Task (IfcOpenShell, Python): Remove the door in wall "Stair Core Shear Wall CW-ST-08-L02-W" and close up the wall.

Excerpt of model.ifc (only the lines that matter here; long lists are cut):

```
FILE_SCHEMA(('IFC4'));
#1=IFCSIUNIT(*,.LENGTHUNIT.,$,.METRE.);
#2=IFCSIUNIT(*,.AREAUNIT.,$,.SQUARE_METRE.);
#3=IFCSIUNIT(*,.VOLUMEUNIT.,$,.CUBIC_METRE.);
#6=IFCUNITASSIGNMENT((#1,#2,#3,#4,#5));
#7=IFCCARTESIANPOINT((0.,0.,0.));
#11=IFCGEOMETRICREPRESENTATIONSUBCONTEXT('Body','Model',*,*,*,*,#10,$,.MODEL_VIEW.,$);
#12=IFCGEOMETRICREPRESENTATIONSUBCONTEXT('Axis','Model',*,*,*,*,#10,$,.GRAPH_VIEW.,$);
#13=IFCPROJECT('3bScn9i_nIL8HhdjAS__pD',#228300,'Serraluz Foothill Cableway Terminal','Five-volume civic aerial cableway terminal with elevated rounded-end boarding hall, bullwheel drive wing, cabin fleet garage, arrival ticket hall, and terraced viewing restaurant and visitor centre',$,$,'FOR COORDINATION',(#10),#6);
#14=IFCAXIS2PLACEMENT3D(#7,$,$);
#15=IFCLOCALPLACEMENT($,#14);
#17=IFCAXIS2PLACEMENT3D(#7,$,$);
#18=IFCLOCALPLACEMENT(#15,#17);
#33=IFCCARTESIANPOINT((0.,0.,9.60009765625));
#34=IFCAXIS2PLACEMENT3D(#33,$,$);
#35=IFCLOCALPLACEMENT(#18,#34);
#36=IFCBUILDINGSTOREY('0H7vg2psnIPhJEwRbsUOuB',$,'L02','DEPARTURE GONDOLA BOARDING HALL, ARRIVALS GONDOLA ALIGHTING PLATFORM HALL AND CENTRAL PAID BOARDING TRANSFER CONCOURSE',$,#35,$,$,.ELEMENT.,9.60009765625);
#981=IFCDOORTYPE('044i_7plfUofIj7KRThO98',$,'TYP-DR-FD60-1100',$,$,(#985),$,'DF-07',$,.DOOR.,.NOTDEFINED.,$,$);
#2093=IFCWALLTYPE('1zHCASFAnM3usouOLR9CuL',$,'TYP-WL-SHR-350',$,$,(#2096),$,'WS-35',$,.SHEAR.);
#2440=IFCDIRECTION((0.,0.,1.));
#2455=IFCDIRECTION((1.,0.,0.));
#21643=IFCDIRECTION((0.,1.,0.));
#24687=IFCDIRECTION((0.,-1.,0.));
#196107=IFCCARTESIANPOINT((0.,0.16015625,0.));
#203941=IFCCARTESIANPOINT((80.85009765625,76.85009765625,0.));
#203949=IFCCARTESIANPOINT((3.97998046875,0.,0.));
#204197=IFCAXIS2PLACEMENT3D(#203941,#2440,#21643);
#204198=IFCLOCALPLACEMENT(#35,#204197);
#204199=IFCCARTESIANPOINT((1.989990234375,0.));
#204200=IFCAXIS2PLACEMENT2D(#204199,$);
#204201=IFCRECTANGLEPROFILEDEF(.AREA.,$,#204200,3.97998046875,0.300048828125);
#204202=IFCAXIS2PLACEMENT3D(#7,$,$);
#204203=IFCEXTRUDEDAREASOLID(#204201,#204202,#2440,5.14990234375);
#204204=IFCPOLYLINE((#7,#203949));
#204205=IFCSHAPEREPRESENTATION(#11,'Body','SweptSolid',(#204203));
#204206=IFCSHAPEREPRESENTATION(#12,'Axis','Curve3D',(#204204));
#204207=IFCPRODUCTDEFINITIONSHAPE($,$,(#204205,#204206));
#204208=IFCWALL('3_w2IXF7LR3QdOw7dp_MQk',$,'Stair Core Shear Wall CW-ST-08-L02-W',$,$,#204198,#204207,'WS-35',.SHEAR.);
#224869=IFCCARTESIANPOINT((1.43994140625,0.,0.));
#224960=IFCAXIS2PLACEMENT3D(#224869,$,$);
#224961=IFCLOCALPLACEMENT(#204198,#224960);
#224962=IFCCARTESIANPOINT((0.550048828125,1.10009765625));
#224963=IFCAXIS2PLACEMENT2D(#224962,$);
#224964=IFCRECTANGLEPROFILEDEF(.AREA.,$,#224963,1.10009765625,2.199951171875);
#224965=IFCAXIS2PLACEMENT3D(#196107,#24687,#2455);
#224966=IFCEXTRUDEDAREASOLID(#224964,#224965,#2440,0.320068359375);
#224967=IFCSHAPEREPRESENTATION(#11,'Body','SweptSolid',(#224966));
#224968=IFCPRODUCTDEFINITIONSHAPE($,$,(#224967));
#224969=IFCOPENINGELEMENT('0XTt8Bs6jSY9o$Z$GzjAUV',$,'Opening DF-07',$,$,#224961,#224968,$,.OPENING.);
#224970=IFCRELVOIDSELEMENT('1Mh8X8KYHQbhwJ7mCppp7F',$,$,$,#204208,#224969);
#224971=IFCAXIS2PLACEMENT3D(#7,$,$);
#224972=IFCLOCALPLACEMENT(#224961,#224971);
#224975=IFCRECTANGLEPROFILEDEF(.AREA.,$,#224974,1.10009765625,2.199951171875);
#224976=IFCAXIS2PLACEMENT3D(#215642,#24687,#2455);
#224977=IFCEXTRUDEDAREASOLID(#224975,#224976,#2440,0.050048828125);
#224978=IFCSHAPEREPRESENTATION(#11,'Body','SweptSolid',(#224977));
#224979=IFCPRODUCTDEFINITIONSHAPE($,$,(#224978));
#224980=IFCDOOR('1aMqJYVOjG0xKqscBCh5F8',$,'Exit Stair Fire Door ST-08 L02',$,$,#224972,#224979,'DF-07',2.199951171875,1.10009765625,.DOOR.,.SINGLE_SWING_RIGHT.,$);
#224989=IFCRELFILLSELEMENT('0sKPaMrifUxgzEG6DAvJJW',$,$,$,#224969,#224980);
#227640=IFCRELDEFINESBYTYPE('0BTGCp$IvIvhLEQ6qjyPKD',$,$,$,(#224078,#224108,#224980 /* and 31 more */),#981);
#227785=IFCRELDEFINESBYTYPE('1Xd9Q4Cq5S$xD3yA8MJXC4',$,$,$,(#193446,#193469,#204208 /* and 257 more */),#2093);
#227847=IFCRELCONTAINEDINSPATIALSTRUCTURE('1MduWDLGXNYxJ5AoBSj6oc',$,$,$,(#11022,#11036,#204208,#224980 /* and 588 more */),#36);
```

```python
import ifcopenshell
import ifcopenshell.api.feature
import ifcopenshell.api.root
import ifcopenshell.geom
import ifcopenshell.util.shape

model = ifcopenshell.open("model.ifc")
settings = ifcopenshell.geom.settings()


def volume(element):
    """Net volume in cubic metres, openings subtracted."""
    shape = ifcopenshell.geom.create_shape(settings, element)
    return ifcopenshell.util.shape.get_volume(shape.geometry)


door = model.by_guid("1aMqJYVOjG0xKqscBCh5F8")
opening = door.FillsVoids[0].RelatingOpeningElement
wall = opening.VoidsElements[0].RelatingBuildingElement
before = volume(wall)

ifcopenshell.api.root.remove_product(model, product=door)
ifcopenshell.api.feature.remove_feature(model, feature=opening)

after = volume(wall)

print(f"wall volume {before:.3f} -> {after:.3f} m3")

model.write("model_updated.ifc")
```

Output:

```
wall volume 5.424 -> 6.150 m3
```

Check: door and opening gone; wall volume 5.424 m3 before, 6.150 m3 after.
